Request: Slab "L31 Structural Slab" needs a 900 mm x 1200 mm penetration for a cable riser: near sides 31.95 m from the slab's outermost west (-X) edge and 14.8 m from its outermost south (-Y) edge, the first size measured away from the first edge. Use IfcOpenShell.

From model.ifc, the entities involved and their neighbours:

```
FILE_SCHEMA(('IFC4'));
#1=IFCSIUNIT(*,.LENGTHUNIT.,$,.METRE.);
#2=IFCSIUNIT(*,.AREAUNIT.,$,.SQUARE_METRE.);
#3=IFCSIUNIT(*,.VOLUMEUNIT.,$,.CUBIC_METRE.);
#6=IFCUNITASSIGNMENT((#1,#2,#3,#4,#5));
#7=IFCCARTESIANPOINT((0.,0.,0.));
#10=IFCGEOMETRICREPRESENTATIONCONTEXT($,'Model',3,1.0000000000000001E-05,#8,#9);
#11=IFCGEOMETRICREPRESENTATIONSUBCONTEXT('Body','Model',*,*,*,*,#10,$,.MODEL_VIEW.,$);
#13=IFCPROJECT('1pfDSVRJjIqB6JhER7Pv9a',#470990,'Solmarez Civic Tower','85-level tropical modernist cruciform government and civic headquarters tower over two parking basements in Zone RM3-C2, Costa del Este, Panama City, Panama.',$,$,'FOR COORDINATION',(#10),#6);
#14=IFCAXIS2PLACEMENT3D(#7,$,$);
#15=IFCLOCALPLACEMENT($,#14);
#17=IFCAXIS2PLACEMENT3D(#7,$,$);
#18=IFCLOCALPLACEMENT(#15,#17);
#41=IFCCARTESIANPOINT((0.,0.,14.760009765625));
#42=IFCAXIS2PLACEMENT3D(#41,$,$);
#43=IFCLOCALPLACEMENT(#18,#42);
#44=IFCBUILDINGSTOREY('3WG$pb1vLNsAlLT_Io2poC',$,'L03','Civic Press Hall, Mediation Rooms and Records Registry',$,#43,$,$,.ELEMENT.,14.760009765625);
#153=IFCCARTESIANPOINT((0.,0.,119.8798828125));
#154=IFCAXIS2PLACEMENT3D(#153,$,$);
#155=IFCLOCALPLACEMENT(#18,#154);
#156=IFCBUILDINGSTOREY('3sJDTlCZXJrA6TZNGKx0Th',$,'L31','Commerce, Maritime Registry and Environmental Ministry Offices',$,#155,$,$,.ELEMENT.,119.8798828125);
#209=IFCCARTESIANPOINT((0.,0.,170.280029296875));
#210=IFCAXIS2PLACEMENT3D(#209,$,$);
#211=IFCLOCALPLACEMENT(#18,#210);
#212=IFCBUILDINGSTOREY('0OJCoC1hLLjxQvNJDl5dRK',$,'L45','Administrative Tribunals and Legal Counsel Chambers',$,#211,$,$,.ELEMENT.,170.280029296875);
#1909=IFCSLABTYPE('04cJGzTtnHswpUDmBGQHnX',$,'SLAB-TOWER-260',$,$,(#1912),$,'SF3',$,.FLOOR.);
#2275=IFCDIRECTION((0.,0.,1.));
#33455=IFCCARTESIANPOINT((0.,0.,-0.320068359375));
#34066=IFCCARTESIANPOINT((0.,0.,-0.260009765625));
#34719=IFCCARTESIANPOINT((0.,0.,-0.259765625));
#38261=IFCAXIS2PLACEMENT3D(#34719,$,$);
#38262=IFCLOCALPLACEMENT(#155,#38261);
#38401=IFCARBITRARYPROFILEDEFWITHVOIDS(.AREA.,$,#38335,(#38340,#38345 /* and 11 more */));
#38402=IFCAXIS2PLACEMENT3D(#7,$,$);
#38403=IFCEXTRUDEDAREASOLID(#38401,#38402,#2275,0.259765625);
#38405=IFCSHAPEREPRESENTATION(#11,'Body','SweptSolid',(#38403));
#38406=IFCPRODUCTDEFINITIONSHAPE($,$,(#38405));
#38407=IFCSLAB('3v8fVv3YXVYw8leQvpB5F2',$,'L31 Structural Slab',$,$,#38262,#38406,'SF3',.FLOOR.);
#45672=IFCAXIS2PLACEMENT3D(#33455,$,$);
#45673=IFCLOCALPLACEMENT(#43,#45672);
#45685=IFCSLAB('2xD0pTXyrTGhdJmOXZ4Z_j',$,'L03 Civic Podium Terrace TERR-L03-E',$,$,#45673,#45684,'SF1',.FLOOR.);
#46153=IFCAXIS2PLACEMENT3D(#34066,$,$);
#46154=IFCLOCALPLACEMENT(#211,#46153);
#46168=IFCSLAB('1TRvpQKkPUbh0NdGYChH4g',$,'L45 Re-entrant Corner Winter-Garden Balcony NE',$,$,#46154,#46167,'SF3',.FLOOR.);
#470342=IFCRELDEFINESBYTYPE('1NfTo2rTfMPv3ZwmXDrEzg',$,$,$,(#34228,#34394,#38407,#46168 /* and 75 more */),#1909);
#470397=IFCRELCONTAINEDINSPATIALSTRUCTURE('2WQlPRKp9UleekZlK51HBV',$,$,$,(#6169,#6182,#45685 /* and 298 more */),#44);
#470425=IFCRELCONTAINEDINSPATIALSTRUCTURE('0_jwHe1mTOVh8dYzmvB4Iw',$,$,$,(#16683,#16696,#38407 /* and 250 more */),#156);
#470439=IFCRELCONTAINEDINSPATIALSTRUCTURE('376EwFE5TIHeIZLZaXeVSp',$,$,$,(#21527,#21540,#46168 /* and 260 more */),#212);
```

```python
import numpy as np
import ifcopenshell
import ifcopenshell.api.feature
import ifcopenshell.api.geometry
import ifcopenshell.api.root
import ifcopenshell.geom
import ifcopenshell.util.placement
import ifcopenshell.util.representation
import ifcopenshell.util.shape
import ifcopenshell.util.unit

model = ifcopenshell.open("model.ifc")
unit_scale = ifcopenshell.util.unit.calculate_unit_scale(model)
settings = ifcopenshell.geom.settings()


def volume(element):
    """Net volume in cubic metres, openings subtracted."""
    shape = ifcopenshell.geom.create_shape(settings, element)
    return ifcopenshell.util.shape.get_volume(shape.geometry)


slab = model.by_id(38407)
before = volume(slab)

# Extent in the slab's own axes, in metres. The edges named are its -X and -Y sides.
slab_shape = ifcopenshell.geom.create_shape(settings, slab)
vertices = ifcopenshell.util.shape.get_vertices(slab_shape.geometry)
x_min, y_min, bottom = vertices.min(axis=0)
top = vertices[:, 2].max()

opening = ifcopenshell.api.root.create_entity(model, ifc_class="IfcOpeningElement", name="Cable riser opening", predefined_type="OPENING")
context = ifcopenshell.util.representation.get_context(model, "Model", "Body", "MODEL_VIEW")
width, depth = 0.9, 1.2
outline = [(0.0, 0.0), (width, 0.0), (width, depth), (0.0, depth), (0.0, 0.0)]
# Overshoot both faces by 50 mm so the cut is clean.
shape = ifcopenshell.api.geometry.add_slab_representation(
    model, context=context, depth=top - bottom + 0.1, polyline=outline
)
ifcopenshell.api.geometry.assign_representation(model, product=opening, representation=shape)

matrix = ifcopenshell.util.placement.get_local_placement(slab.ObjectPlacement)
matrix[:, 3] = matrix @ np.append(np.array([x_min + 31.95, y_min + 14.8, bottom - 0.05]) / unit_scale, 1.0)
ifcopenshell.api.geometry.edit_object_placement(model, product=opening, matrix=matrix, is_si=False)
ifcopenshell.api.feature.add_feature(model, feature=opening, element=slab)

after = volume(slab)

print(f"slab volume {before:.3f} -> {after:.3f} m3")

model.write("model_v2.ifc")
```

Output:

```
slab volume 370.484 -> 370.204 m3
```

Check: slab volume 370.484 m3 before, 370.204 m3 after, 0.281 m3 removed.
